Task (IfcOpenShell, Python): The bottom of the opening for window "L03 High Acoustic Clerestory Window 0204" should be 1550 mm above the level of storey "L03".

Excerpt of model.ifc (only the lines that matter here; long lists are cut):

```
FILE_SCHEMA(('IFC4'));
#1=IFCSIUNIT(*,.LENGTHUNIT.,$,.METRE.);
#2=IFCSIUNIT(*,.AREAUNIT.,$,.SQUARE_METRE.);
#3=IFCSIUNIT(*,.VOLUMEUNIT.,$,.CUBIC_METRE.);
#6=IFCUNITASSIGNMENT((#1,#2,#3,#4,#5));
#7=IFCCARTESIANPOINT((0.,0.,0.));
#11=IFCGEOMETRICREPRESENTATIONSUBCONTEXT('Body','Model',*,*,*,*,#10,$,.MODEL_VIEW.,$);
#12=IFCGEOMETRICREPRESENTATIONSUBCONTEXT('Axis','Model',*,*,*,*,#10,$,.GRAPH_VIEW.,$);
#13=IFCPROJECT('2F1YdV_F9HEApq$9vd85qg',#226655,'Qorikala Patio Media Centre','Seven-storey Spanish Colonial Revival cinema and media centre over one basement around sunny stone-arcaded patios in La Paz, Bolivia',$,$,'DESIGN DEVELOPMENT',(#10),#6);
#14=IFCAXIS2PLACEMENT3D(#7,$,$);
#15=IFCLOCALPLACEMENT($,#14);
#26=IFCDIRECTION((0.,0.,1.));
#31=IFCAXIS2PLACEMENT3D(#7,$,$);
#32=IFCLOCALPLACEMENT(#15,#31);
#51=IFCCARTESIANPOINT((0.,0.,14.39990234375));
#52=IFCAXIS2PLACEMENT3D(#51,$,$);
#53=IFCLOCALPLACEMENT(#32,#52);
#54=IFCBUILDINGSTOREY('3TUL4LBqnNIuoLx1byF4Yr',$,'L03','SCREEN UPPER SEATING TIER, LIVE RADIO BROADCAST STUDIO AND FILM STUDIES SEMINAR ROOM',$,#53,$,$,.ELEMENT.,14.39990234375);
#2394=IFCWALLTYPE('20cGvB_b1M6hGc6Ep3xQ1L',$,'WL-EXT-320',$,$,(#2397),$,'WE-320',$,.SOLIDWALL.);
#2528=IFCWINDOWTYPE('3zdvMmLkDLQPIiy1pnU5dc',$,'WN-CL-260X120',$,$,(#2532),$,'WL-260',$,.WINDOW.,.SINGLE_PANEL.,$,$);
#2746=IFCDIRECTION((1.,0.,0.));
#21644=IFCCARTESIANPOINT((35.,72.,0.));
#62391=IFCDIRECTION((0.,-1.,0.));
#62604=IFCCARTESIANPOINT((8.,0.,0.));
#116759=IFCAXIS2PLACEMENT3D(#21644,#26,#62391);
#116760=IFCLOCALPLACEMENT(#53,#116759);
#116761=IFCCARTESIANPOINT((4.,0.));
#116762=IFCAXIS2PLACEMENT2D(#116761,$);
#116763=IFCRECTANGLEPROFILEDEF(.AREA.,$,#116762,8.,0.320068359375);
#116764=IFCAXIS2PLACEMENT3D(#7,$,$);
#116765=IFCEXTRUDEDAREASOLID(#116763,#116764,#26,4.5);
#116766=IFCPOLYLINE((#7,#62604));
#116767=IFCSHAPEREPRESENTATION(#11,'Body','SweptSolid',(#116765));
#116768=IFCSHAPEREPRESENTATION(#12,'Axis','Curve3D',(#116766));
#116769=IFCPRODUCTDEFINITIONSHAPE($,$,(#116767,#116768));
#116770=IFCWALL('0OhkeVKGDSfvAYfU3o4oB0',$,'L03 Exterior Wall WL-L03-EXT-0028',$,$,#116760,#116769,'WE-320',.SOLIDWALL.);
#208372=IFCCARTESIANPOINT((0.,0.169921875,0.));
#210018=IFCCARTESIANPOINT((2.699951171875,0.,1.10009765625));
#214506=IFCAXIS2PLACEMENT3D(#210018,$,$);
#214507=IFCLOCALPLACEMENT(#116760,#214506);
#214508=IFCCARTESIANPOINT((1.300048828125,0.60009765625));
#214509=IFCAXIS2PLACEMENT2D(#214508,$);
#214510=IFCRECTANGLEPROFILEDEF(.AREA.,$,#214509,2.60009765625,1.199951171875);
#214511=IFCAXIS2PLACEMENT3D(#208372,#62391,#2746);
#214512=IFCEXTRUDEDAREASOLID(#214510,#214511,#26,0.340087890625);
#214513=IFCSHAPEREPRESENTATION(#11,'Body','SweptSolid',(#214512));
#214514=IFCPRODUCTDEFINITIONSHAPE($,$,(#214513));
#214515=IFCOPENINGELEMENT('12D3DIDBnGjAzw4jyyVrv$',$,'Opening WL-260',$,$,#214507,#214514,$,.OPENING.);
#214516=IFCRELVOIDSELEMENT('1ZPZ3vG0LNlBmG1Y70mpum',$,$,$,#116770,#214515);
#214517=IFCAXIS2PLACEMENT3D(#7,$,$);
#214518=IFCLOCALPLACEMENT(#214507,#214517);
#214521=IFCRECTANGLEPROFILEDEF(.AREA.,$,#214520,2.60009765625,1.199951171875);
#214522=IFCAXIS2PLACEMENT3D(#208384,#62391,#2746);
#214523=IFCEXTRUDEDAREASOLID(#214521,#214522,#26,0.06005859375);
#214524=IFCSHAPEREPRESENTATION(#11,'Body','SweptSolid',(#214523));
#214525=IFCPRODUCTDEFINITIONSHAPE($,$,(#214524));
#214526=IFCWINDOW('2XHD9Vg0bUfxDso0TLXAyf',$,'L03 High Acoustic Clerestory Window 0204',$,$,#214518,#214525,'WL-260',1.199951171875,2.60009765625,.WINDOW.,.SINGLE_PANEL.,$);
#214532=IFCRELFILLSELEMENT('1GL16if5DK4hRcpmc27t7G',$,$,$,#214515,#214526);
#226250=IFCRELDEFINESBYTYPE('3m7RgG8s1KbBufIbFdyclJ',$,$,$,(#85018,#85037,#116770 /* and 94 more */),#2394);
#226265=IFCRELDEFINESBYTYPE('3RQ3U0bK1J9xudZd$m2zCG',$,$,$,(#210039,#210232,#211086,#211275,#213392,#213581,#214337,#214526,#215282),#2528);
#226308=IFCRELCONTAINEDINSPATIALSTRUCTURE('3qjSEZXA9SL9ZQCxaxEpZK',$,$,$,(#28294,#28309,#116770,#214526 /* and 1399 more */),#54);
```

```python
import numpy as np
import ifcopenshell
import ifcopenshell.api.geometry
import ifcopenshell.geom
import ifcopenshell.util.element
import ifcopenshell.util.placement
import ifcopenshell.util.shape
import ifcopenshell.util.unit

model = ifcopenshell.open("model.ifc")
unit_scale = ifcopenshell.util.unit.calculate_unit_scale(model)

window = model.by_guid("2XHD9Vg0bUfxDso0TLXAyf")
opening = window.FillsVoids[0].RelatingOpeningElement
storey = ifcopenshell.util.element.get_container(window, ifc_class="IfcBuildingStorey")
level = ifcopenshell.util.placement.get_local_placement(storey.ObjectPlacement)[2, 3]

# The opening's origin need not be at the sill, so measure its lowest point.
shape = ifcopenshell.geom.create_shape(ifcopenshell.geom.settings(), opening)
bottom = ifcopenshell.util.shape.get_shape_bottom_elevation(shape, shape.geometry) / unit_scale
dz = level + 1.55 / unit_scale - bottom

shift = np.array([0.0, 0.0, dz])
# The window is placed relative to its opening, so it follows when the opening moves.
matrix = ifcopenshell.util.placement.get_local_placement(opening.ObjectPlacement)
matrix[:3, 3] += shift
ifcopenshell.api.geometry.edit_object_placement(
    model, product=opening, matrix=matrix, is_si=False, should_transform_children=True
)

print(f"moved by {dz * unit_scale:+.3f} m")

model.write("model_v2.ifc")
```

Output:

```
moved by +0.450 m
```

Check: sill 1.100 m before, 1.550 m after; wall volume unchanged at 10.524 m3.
